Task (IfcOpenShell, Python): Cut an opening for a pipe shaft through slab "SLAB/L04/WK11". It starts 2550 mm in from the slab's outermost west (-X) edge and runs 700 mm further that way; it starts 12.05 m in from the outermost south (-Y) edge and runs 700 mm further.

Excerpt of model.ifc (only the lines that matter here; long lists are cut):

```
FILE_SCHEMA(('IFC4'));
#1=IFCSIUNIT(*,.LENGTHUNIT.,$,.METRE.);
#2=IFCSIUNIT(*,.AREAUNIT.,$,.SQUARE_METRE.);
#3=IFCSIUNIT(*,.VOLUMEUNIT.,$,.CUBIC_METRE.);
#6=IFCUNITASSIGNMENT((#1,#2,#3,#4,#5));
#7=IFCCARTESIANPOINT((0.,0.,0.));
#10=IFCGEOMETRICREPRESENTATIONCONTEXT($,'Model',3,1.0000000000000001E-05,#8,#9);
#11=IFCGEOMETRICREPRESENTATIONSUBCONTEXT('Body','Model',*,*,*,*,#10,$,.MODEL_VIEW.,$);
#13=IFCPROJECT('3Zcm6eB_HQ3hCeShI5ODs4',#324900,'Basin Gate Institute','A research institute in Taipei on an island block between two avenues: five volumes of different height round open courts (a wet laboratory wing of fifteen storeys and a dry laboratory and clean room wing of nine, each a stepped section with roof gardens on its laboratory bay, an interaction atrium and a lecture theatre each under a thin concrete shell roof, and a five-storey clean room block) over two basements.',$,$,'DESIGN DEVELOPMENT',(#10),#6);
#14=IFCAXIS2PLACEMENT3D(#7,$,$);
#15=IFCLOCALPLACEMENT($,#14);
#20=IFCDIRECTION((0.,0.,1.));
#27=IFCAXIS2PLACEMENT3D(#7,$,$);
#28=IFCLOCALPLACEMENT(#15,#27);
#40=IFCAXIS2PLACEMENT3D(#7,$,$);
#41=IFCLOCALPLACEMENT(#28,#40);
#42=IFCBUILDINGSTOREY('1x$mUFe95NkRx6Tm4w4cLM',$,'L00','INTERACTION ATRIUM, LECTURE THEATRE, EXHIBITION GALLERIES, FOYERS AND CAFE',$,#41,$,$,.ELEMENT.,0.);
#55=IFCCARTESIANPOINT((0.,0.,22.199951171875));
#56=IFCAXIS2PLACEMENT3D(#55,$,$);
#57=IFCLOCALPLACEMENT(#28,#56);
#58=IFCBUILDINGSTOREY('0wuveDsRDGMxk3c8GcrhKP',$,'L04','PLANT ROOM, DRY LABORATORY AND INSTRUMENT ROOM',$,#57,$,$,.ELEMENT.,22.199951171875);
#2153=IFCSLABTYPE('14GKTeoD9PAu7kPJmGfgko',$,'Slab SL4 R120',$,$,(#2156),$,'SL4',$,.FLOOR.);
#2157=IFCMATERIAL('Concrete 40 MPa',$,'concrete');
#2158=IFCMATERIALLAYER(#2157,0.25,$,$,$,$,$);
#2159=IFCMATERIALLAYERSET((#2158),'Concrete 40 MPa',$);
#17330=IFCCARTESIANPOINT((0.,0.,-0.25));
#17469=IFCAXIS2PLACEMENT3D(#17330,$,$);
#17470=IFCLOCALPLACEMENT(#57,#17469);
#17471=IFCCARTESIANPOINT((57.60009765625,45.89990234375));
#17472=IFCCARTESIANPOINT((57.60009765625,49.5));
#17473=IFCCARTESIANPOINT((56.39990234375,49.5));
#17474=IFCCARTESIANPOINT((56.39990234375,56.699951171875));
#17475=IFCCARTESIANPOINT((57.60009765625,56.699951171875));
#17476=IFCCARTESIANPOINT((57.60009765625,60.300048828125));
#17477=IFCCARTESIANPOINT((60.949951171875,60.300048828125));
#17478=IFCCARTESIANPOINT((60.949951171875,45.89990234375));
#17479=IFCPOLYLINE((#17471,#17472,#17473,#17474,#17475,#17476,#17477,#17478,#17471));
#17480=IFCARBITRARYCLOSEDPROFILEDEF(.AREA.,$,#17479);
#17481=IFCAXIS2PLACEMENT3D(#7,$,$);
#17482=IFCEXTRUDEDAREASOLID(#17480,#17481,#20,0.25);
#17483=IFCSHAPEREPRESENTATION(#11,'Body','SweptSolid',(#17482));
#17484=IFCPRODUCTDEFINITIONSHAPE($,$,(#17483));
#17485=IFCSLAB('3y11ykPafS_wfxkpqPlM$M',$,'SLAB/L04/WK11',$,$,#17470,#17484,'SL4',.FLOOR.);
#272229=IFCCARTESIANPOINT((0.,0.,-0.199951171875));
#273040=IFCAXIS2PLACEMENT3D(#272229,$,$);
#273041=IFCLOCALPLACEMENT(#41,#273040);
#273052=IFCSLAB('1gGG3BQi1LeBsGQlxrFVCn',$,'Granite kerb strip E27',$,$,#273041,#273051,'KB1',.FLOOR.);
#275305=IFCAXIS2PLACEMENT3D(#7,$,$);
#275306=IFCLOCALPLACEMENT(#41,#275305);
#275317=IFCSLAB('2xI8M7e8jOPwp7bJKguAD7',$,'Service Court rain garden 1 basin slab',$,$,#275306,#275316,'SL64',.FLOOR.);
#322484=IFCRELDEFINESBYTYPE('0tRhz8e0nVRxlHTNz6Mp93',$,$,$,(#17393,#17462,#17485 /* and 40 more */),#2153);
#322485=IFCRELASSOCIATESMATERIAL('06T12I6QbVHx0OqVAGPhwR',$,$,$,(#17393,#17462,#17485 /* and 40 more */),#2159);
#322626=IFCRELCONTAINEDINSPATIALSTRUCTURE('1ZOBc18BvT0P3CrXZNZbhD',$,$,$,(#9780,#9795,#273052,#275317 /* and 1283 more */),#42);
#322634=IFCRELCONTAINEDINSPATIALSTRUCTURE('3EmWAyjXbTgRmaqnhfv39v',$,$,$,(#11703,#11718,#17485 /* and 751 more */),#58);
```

```python
import numpy as np
import ifcopenshell
import ifcopenshell.api.feature
import ifcopenshell.api.geometry
import ifcopenshell.api.root
import ifcopenshell.geom
import ifcopenshell.util.placement
import ifcopenshell.util.representation
import ifcopenshell.util.shape
import ifcopenshell.util.unit

model = ifcopenshell.open("model.ifc")
unit_scale = ifcopenshell.util.unit.calculate_unit_scale(model)
settings = ifcopenshell.geom.settings()


def volume(element):
    """Net volume in cubic metres, openings subtracted."""
    shape = ifcopenshell.geom.create_shape(settings, element)
    return ifcopenshell.util.shape.get_volume(shape.geometry)


slab = model.by_guid("3y11ykPafS_wfxkpqPlM$M")
before = volume(slab)

# Extent in the slab's own axes, in metres. The edges named are its -X and -Y sides.
slab_shape = ifcopenshell.geom.create_shape(settings, slab)
vertices = ifcopenshell.util.shape.get_vertices(slab_shape.geometry)
x_min, y_min, bottom = vertices.min(axis=0)
top = vertices[:, 2].max()

opening = ifcopenshell.api.root.create_entity(model, ifc_class="IfcOpeningElement", name="Pipe shaft opening", predefined_type="OPENING")
context = ifcopenshell.util.representation.get_context(model, "Model", "Body", "MODEL_VIEW")
width, depth = 0.7, 0.7
outline = [(0.0, 0.0), (width, 0.0), (width, depth), (0.0, depth), (0.0, 0.0)]
# Overshoot both faces by 50 mm so the cut is clean.
shape = ifcopenshell.api.geometry.add_slab_representation(
    model, context=context, depth=top - bottom + 0.1, polyline=outline
)
ifcopenshell.api.geometry.assign_representation(model, product=opening, representation=shape)

matrix = ifcopenshell.util.placement.get_local_placement(slab.ObjectPlacement)
matrix[:, 3] = matrix @ np.append(np.array([x_min + 2.55, y_min + 12.05, bottom - 0.05]) / unit_scale, 1.0)
ifcopenshell.api.geometry.edit_object_placement(model, product=opening, matrix=matrix, is_si=False)
ifcopenshell.api.feature.add_feature(model, feature=opening, element=slab)

after = volume(slab)

print(f"slab volume {before:.3f} -> {after:.3f} m3")

model.write("model_edited.ifc")
```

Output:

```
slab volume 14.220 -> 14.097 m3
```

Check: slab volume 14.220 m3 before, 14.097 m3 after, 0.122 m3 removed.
